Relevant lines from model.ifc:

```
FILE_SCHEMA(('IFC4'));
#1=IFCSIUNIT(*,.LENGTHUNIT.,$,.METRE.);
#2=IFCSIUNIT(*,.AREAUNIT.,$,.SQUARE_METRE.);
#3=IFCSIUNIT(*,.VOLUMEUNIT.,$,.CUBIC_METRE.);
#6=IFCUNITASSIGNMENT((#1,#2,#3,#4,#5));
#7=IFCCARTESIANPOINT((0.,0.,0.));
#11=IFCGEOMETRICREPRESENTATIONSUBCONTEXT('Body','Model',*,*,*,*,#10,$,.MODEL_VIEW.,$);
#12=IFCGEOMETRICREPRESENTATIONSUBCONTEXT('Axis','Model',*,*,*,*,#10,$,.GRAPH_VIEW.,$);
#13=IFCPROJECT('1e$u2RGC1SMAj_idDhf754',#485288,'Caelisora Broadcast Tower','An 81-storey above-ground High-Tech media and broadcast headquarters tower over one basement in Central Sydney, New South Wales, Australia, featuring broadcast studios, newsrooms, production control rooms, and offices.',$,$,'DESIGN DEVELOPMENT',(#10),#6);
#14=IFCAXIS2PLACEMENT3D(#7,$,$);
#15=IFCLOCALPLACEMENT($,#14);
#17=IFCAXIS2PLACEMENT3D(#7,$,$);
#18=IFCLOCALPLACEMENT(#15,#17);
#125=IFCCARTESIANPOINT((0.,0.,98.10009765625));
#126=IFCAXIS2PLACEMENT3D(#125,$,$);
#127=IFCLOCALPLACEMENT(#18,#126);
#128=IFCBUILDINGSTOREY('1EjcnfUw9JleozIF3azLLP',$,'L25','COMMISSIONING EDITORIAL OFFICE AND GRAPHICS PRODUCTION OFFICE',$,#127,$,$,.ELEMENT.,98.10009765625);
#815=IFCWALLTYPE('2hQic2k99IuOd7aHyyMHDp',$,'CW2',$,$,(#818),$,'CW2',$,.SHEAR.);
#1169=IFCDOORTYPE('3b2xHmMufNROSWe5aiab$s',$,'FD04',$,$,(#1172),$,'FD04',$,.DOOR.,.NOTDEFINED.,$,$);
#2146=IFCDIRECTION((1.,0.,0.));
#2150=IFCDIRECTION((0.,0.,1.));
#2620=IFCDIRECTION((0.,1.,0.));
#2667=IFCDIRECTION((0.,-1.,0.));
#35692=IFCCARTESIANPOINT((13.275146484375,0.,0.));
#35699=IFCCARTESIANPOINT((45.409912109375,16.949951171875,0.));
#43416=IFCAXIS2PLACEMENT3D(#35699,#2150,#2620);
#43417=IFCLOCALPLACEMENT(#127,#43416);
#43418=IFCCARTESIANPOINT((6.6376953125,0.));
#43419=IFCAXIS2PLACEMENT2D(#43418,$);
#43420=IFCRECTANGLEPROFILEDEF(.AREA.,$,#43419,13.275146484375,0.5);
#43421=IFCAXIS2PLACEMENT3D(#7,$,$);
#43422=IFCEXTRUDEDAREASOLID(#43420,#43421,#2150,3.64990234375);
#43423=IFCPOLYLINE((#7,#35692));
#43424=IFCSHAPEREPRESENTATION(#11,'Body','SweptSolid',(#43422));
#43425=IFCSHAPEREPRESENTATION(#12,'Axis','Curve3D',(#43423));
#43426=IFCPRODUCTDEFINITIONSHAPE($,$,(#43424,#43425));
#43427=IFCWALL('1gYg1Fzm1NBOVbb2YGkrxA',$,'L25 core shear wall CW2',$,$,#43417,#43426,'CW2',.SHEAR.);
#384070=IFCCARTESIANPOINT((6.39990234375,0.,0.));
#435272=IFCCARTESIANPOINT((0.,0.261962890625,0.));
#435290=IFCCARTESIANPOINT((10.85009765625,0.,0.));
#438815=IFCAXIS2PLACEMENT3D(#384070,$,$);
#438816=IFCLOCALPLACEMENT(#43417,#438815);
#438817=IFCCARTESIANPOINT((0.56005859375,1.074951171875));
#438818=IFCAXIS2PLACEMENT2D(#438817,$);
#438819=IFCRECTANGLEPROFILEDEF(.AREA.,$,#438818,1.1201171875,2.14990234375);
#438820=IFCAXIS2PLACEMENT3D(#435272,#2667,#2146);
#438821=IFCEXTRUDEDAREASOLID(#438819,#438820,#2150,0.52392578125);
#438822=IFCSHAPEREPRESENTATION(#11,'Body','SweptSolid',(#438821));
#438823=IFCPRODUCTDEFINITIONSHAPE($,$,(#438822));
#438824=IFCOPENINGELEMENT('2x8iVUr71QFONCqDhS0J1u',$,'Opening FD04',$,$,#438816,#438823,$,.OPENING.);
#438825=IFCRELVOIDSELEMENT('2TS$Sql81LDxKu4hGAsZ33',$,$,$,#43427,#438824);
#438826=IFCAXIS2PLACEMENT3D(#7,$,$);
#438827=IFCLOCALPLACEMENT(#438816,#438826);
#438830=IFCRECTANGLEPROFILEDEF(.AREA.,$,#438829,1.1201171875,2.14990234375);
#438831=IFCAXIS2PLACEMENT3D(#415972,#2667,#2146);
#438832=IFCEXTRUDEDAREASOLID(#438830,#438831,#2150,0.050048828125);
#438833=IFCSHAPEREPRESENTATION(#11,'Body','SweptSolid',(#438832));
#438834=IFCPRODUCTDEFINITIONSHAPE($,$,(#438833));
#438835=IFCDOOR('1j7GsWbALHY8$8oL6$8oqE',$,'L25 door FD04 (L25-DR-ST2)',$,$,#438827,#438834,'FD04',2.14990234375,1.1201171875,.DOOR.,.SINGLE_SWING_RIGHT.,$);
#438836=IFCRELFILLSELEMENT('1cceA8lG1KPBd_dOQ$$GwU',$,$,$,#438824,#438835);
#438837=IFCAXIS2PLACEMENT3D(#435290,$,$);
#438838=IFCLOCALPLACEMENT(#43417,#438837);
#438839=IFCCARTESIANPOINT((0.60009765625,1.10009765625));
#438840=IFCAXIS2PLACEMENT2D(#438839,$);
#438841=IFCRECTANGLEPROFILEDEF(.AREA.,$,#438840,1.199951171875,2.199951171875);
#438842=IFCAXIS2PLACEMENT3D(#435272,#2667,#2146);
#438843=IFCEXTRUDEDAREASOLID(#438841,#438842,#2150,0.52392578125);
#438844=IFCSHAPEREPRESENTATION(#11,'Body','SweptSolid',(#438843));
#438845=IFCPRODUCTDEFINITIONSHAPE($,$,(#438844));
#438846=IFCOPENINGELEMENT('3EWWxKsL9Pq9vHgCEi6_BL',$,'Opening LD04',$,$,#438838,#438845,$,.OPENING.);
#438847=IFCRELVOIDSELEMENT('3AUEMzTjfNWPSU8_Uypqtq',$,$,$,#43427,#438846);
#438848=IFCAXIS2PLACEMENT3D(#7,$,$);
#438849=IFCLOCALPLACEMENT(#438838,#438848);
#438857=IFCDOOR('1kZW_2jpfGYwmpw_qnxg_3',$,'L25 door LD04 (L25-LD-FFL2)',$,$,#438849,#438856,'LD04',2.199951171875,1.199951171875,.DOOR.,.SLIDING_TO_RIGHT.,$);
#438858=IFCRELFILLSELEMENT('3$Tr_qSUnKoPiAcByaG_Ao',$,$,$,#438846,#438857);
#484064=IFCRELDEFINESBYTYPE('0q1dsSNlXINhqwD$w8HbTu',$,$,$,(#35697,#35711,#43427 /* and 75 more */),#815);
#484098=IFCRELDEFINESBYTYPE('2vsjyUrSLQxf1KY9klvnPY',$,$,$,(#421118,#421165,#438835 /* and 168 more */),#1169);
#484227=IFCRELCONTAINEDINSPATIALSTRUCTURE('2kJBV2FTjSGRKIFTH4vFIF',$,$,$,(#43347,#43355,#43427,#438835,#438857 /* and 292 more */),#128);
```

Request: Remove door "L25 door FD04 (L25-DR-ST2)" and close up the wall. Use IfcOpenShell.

```python
import ifcopenshell
import ifcopenshell.api.feature
import ifcopenshell.api.root
import ifcopenshell.geom
import ifcopenshell.util.shape

model = ifcopenshell.open("model.ifc")
settings = ifcopenshell.geom.settings()


def volume(element):
    """Net volume in cubic metres, openings subtracted."""
    shape = ifcopenshell.geom.create_shape(settings, element)
    return ifcopenshell.util.shape.get_volume(shape.geometry)


door = model.by_id(438835)
opening = door.FillsVoids[0].RelatingOpeningElement
wall = opening.VoidsElements[0].RelatingBuildingElement
before = volume(wall)

ifcopenshell.api.root.remove_product(model, product=door)
ifcopenshell.api.feature.remove_feature(model, feature=opening)

after = volume(wall)

print(f"wall volume {before:.3f} -> {after:.3f} m3")

model.write("model_updated.ifc")
```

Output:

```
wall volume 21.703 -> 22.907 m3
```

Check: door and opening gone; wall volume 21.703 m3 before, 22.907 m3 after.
